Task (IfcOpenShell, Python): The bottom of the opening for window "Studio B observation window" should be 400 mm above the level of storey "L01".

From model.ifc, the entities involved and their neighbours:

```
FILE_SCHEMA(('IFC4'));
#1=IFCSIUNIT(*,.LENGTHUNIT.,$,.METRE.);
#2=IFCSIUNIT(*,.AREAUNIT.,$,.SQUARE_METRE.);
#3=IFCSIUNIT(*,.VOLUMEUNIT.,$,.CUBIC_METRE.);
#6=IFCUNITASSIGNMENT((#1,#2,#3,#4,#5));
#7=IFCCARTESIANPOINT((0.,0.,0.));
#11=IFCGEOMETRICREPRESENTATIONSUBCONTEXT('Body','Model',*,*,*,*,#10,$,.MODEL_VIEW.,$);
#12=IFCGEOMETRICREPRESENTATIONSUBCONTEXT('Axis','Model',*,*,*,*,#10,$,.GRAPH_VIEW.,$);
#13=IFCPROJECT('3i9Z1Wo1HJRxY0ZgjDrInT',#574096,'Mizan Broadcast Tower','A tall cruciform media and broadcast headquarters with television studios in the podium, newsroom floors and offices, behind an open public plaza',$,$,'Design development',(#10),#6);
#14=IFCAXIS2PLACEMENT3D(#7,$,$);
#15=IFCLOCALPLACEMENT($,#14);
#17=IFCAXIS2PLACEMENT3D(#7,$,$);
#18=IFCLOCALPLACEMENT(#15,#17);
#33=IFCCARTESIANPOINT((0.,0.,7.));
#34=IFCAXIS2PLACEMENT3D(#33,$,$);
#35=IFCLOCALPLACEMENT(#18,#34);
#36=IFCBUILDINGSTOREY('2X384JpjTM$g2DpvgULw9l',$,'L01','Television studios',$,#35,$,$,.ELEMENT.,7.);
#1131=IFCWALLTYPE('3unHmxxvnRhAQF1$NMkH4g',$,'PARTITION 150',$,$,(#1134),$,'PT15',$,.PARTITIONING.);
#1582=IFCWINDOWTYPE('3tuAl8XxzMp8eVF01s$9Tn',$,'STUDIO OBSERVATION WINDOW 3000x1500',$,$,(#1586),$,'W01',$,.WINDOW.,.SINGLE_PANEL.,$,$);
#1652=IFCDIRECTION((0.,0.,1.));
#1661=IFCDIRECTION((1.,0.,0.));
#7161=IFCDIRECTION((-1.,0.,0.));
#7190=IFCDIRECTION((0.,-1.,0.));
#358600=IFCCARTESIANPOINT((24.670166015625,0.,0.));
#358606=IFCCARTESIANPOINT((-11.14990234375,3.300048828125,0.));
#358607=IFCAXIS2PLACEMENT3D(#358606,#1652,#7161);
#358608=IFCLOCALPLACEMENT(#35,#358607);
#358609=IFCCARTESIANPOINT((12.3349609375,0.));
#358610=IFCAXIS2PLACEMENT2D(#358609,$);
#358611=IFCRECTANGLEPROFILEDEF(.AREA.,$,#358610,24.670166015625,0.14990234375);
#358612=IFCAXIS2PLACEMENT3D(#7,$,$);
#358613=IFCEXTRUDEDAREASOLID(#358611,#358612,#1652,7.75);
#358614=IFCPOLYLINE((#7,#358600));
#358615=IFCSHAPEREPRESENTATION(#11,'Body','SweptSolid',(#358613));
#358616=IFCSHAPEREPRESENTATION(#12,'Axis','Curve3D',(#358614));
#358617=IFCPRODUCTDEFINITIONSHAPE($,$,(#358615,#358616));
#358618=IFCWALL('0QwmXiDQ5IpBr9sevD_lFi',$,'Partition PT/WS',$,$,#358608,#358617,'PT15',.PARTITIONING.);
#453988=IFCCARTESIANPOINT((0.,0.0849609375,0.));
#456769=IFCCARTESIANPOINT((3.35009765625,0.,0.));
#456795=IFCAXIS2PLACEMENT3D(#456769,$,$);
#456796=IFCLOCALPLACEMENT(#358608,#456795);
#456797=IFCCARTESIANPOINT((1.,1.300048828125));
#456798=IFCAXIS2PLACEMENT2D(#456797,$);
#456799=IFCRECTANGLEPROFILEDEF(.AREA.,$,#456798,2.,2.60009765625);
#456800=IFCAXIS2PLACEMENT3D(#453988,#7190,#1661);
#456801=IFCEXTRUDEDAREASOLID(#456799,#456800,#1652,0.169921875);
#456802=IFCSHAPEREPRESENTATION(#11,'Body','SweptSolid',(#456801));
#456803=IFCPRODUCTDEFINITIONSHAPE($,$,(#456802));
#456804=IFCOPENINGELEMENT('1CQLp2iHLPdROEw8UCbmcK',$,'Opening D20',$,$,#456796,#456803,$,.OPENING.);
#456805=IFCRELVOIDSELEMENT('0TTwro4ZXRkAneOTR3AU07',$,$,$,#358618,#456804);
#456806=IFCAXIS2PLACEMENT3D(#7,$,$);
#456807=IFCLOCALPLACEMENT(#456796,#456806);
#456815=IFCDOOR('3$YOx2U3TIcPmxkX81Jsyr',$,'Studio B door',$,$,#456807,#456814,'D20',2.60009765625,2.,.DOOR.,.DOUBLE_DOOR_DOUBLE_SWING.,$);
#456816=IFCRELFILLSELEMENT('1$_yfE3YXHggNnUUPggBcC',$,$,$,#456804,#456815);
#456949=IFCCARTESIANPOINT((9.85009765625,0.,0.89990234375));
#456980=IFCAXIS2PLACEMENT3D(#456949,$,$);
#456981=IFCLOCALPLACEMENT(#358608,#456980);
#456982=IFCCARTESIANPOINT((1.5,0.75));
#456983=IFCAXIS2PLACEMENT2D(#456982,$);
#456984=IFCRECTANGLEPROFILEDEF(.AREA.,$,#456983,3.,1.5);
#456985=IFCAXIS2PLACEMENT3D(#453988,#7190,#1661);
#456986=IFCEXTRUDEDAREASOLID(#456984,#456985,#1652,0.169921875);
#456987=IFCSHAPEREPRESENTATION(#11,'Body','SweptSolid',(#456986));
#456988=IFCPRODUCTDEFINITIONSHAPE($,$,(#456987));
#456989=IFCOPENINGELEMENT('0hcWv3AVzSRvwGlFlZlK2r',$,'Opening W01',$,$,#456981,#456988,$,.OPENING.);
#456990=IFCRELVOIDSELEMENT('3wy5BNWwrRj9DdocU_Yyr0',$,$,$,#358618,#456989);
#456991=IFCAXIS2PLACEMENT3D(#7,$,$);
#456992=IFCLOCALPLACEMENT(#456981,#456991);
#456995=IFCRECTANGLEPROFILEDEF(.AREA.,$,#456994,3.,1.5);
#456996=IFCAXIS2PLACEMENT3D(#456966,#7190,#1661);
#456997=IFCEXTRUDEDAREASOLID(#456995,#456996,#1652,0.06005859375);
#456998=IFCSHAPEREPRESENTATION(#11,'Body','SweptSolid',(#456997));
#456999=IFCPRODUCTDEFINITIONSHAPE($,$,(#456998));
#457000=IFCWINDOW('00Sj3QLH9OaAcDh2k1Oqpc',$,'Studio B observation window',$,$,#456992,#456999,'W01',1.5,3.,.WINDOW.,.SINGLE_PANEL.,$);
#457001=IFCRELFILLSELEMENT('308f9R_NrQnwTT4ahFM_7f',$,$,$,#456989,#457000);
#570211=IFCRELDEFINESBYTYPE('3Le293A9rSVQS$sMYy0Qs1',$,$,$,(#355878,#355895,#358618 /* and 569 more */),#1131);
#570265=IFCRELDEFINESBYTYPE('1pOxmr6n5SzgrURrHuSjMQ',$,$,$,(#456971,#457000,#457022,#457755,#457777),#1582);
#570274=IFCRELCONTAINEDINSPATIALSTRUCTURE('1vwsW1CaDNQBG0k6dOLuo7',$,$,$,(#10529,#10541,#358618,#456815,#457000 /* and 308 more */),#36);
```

```python
import numpy as np
import ifcopenshell
import ifcopenshell.api.geometry
import ifcopenshell.geom
import ifcopenshell.util.element
import ifcopenshell.util.placement
import ifcopenshell.util.shape
import ifcopenshell.util.unit

model = ifcopenshell.open("model.ifc")
unit_scale = ifcopenshell.util.unit.calculate_unit_scale(model)

window = model.by_guid("00Sj3QLH9OaAcDh2k1Oqpc")
opening = window.FillsVoids[0].RelatingOpeningElement
storey = ifcopenshell.util.element.get_container(window, ifc_class="IfcBuildingStorey")
level = ifcopenshell.util.placement.get_local_placement(storey.ObjectPlacement)[2, 3]

# The opening's origin need not be at the sill, so measure its lowest point.
shape = ifcopenshell.geom.create_shape(ifcopenshell.geom.settings(), opening)
bottom = ifcopenshell.util.shape.get_shape_bottom_elevation(shape, shape.geometry) / unit_scale
dz = level + 0.4 - bottom

shift = np.array([0.0, 0.0, dz])
# The window is placed relative to its opening, so it follows when the opening moves.
matrix = ifcopenshell.util.placement.get_local_placement(opening.ObjectPlacement)
matrix[:3, 3] += shift
ifcopenshell.api.geometry.edit_object_placement(
    model, product=opening, matrix=matrix, is_si=False, should_transform_children=True
)

print(f"moved by {dz * unit_scale:+.3f} m")

model.write("model_v2.ifc")
```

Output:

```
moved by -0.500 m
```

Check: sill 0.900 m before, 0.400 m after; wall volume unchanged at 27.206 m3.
